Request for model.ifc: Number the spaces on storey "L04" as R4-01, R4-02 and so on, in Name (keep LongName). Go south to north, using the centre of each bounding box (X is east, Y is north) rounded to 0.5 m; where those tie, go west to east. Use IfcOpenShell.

First a look at what the model holds.

```python
import ifcopenshell
import ifcopenshell.util.element
import ifcopenshell.util.placement

model = ifcopenshell.open("model.ifc")
print(model.schema)
storey = next(s for s in model.by_type("IfcBuildingStorey") if s.Name == "L04")
spaces = [e for e in ifcopenshell.util.element.get_decomposition(storey) if e.is_a("IfcSpace")]
for e in sorted(spaces, key=lambda e: e.id()):
    origin = ifcopenshell.util.placement.get_local_placement(e.ObjectPlacement)[:3, 3]
    print(e.id(), e.Name, e.LongName, origin.round(2) + 0.0, sep=" | ")
```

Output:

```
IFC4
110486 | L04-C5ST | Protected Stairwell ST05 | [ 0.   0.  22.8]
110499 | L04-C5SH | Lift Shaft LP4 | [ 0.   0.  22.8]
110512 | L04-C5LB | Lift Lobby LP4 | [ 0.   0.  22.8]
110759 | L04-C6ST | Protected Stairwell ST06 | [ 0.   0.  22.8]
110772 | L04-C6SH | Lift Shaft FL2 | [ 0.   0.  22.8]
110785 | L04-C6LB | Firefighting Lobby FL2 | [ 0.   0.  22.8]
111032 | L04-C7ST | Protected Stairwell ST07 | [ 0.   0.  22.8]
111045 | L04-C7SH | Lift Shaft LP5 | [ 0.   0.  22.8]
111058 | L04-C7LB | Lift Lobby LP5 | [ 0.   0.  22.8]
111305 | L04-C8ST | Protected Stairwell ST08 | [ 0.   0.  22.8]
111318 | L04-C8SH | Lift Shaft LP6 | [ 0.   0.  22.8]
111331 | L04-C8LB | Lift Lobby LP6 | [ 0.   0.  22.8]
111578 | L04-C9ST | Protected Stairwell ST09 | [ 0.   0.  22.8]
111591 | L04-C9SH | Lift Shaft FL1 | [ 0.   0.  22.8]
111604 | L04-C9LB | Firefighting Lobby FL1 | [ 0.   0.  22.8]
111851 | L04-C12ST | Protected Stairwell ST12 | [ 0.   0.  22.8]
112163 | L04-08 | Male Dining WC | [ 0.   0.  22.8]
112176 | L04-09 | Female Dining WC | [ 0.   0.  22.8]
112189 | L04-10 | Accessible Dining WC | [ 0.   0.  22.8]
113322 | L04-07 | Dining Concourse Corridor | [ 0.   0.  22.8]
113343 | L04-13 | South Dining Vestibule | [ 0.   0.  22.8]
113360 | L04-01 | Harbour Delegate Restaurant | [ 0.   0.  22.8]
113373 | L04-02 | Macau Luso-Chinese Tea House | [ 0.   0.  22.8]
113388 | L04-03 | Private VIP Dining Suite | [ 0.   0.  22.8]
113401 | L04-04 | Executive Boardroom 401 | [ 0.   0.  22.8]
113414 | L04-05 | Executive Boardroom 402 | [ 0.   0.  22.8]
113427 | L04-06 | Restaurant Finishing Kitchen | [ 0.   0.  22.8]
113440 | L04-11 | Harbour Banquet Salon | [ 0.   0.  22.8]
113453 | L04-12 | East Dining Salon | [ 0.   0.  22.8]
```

```python
import ifcopenshell
import ifcopenshell.geom
import ifcopenshell.util.element
import ifcopenshell.util.shape

model = ifcopenshell.open("model.ifc")
settings = ifcopenshell.geom.settings()
settings.set("use-world-coords", True)


def centre(element):
    shape = ifcopenshell.geom.create_shape(settings, element)
    return ifcopenshell.util.shape.get_bbox_centroid(shape.geometry)


storey = next(s for s in model.by_type("IfcBuildingStorey") if s.Name == "L04")
spaces = [e for e in ifcopenshell.util.element.get_decomposition(storey) if e.is_a("IfcSpace")]

# Insertion points can sit at a corner or the storey origin, so sort by the geometry (in metres).
centres = {e: centre(e) for e in spaces}
spaces.sort(key=lambda e: (round(centres[e][1] / 0.5), centres[e][0]))

for i, e in enumerate(spaces, start=1):
    number = f"R4-{i:02d}"
    e.Name = number
    print(e.id(), number)

model.write("model_edited.ifc")
```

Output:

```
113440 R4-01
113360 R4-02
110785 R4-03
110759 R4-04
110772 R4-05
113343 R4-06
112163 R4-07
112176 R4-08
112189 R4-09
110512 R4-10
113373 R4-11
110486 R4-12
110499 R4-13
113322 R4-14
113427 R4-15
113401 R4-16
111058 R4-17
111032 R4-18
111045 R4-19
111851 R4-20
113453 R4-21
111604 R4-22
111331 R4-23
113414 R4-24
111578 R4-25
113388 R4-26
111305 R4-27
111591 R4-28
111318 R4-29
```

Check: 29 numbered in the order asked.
